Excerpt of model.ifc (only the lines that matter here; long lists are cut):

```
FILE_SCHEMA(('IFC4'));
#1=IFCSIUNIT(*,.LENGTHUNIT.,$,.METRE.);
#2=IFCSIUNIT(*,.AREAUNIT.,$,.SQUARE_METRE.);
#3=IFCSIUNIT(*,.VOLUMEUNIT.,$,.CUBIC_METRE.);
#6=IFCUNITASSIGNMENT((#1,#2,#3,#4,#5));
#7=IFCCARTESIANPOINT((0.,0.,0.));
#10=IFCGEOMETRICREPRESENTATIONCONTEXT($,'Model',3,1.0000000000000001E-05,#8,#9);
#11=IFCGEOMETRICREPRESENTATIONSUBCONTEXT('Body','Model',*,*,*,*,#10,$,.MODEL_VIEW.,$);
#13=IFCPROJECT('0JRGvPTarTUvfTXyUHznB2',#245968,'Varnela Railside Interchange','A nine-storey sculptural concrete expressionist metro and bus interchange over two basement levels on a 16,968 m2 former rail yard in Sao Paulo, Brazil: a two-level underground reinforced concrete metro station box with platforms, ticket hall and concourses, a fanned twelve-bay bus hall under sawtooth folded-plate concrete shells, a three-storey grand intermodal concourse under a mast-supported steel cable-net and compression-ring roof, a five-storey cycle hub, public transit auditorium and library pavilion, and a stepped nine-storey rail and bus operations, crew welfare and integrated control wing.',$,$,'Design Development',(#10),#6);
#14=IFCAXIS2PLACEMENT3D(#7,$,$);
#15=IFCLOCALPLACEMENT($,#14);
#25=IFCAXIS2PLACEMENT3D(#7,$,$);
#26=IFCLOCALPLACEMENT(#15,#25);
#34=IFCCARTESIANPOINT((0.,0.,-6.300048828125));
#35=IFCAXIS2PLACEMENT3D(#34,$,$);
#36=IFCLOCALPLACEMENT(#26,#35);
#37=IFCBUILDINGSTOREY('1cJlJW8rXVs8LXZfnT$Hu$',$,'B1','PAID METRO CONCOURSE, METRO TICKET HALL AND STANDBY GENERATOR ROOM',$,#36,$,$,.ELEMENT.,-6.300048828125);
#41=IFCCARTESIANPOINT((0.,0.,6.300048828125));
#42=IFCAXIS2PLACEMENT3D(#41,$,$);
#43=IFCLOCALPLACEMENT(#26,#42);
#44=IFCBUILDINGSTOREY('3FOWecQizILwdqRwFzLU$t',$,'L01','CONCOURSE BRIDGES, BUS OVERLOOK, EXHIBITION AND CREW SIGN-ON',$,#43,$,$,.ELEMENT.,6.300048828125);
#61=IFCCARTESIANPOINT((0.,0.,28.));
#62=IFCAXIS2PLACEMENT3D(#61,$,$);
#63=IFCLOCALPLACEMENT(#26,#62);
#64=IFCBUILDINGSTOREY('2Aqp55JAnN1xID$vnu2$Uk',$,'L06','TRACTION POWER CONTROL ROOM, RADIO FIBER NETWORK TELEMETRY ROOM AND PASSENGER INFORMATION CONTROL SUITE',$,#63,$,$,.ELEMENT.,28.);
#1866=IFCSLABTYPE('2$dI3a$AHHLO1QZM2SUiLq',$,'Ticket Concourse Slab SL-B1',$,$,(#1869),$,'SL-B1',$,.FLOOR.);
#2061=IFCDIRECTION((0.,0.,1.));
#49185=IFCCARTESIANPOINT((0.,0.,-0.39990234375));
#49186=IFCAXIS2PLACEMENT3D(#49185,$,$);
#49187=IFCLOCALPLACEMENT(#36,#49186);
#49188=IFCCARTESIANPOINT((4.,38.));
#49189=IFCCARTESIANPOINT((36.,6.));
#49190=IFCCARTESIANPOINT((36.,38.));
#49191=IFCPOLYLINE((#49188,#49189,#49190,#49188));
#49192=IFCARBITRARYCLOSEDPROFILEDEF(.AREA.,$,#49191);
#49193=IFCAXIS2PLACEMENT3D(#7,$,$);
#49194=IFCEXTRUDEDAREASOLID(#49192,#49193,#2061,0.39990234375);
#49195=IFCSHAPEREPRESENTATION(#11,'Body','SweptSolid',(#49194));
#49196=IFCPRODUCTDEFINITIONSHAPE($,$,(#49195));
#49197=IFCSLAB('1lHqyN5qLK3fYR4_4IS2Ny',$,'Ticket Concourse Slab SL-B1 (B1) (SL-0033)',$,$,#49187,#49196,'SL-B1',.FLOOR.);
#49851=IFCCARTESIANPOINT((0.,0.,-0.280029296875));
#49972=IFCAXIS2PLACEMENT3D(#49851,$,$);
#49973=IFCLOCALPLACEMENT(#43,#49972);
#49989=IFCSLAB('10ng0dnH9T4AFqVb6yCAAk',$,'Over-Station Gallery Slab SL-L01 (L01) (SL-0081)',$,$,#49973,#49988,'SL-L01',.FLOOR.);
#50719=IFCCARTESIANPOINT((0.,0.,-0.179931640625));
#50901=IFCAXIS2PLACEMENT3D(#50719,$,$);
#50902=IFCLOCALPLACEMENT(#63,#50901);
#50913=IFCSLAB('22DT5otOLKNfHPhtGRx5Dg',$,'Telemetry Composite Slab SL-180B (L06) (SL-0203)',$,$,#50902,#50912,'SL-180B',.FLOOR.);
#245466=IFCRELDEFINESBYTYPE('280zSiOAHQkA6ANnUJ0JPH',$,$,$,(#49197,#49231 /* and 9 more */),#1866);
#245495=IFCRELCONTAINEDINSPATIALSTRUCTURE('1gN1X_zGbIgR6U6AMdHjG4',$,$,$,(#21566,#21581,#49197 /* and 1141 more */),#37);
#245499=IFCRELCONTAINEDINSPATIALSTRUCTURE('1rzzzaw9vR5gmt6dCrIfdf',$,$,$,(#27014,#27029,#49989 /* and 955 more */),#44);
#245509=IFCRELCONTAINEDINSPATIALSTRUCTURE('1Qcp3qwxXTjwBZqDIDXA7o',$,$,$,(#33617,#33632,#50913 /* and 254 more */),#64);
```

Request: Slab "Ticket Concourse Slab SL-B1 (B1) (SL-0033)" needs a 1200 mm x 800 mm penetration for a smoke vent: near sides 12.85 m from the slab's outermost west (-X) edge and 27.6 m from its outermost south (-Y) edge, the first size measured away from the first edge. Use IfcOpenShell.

```python
import numpy as np
import ifcopenshell
import ifcopenshell.api.feature
import ifcopenshell.api.geometry
import ifcopenshell.api.root
import ifcopenshell.geom
import ifcopenshell.util.placement
import ifcopenshell.util.representation
import ifcopenshell.util.shape
import ifcopenshell.util.unit

model = ifcopenshell.open("model.ifc")
unit_scale = ifcopenshell.util.unit.calculate_unit_scale(model)
settings = ifcopenshell.geom.settings()


def volume(element):
    """Net volume in cubic metres, openings subtracted."""
    shape = ifcopenshell.geom.create_shape(settings, element)
    return ifcopenshell.util.shape.get_volume(shape.geometry)


slab = model.by_id(49197)
before = volume(slab)

# Extent in the slab's own axes, in metres. The edges named are its -X and -Y sides.
slab_shape = ifcopenshell.geom.create_shape(settings, slab)
vertices = ifcopenshell.util.shape.get_vertices(slab_shape.geometry)
x_min, y_min, bottom = vertices.min(axis=0)
top = vertices[:, 2].max()

opening = ifcopenshell.api.root.create_entity(model, ifc_class="IfcOpeningElement", name="Smoke vent opening", predefined_type="OPENING")
context = ifcopenshell.util.representation.get_context(model, "Model", "Body", "MODEL_VIEW")
width, depth = 1.2, 0.8
outline = [(0.0, 0.0), (width, 0.0), (width, depth), (0.0, depth), (0.0, 0.0)]
# Overshoot both faces by 50 mm so the cut is clean.
shape = ifcopenshell.api.geometry.add_slab_representation(
    model, context=context, depth=top - bottom + 0.1, polyline=outline
)
ifcopenshell.api.geometry.assign_representation(model, product=opening, representation=shape)

matrix = ifcopenshell.util.placement.get_local_placement(slab.ObjectPlacement)
matrix[:, 3] = matrix @ np.append(np.array([x_min + 12.85, y_min + 27.6, bottom - 0.05]) / unit_scale, 1.0)
ifcopenshell.api.geometry.edit_object_placement(model, product=opening, matrix=matrix, is_si=False)
ifcopenshell.api.feature.add_feature(model, feature=opening, element=slab)

after = volume(slab)

print(f"slab volume {before:.3f} -> {after:.3f} m3")

model.write("model_v2.ifc")
```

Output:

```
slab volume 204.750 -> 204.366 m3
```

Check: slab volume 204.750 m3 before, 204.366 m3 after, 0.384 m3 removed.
